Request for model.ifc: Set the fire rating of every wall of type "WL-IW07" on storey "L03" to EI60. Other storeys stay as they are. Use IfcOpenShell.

First a look at what the model holds.

```python
import ifcopenshell
import ifcopenshell.util.element

model = ifcopenshell.open("model.ifc")
print(model.schema)
storey = next(s for s in model.by_type("IfcBuildingStorey") if s.Name == "L03")
walls = [e for e in ifcopenshell.util.element.get_decomposition(storey) if e.is_a("IfcWall")]
seen = {}
for e in walls:
    element_type = ifcopenshell.util.element.get_type(e)
    key = (element_type.Name if element_type != e and element_type else None, ifcopenshell.util.element.get_pset(e, "Pset_WallCommon", "FireRating"))
    seen[key] = seen.get(key, 0) + 1
for (name, value), count in sorted(seen.items(), key=str):
    print(count, "x", name, "|", value)
```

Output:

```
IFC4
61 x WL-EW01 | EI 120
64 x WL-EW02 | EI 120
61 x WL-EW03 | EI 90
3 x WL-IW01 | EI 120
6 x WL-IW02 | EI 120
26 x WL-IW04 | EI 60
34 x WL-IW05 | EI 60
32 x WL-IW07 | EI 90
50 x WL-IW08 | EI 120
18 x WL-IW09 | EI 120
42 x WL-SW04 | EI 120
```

```python
import ifcopenshell
import ifcopenshell.api.pset
import ifcopenshell.util.element

model = ifcopenshell.open("model.ifc")

storey = next(s for s in model.by_type("IfcBuildingStorey") if s.Name == "L03")
walls = [e for e in ifcopenshell.util.element.get_decomposition(storey) if e.is_a("IfcWall")]

count = 0
for e in walls:
    element_type = ifcopenshell.util.element.get_type(e)
    if element_type in (None, e) or element_type.Name != "WL-IW07":
        continue
    # add_pset returns the element's existing set when there is one.
    pset = ifcopenshell.api.pset.add_pset(model, product=e, name="Pset_WallCommon")
    ifcopenshell.api.pset.edit_pset(model, pset=pset, properties={"FireRating": "EI60"})
    count += 1

print(count, "walls updated")

model.write("model-out.ifc")
```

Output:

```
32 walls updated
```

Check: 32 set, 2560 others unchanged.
